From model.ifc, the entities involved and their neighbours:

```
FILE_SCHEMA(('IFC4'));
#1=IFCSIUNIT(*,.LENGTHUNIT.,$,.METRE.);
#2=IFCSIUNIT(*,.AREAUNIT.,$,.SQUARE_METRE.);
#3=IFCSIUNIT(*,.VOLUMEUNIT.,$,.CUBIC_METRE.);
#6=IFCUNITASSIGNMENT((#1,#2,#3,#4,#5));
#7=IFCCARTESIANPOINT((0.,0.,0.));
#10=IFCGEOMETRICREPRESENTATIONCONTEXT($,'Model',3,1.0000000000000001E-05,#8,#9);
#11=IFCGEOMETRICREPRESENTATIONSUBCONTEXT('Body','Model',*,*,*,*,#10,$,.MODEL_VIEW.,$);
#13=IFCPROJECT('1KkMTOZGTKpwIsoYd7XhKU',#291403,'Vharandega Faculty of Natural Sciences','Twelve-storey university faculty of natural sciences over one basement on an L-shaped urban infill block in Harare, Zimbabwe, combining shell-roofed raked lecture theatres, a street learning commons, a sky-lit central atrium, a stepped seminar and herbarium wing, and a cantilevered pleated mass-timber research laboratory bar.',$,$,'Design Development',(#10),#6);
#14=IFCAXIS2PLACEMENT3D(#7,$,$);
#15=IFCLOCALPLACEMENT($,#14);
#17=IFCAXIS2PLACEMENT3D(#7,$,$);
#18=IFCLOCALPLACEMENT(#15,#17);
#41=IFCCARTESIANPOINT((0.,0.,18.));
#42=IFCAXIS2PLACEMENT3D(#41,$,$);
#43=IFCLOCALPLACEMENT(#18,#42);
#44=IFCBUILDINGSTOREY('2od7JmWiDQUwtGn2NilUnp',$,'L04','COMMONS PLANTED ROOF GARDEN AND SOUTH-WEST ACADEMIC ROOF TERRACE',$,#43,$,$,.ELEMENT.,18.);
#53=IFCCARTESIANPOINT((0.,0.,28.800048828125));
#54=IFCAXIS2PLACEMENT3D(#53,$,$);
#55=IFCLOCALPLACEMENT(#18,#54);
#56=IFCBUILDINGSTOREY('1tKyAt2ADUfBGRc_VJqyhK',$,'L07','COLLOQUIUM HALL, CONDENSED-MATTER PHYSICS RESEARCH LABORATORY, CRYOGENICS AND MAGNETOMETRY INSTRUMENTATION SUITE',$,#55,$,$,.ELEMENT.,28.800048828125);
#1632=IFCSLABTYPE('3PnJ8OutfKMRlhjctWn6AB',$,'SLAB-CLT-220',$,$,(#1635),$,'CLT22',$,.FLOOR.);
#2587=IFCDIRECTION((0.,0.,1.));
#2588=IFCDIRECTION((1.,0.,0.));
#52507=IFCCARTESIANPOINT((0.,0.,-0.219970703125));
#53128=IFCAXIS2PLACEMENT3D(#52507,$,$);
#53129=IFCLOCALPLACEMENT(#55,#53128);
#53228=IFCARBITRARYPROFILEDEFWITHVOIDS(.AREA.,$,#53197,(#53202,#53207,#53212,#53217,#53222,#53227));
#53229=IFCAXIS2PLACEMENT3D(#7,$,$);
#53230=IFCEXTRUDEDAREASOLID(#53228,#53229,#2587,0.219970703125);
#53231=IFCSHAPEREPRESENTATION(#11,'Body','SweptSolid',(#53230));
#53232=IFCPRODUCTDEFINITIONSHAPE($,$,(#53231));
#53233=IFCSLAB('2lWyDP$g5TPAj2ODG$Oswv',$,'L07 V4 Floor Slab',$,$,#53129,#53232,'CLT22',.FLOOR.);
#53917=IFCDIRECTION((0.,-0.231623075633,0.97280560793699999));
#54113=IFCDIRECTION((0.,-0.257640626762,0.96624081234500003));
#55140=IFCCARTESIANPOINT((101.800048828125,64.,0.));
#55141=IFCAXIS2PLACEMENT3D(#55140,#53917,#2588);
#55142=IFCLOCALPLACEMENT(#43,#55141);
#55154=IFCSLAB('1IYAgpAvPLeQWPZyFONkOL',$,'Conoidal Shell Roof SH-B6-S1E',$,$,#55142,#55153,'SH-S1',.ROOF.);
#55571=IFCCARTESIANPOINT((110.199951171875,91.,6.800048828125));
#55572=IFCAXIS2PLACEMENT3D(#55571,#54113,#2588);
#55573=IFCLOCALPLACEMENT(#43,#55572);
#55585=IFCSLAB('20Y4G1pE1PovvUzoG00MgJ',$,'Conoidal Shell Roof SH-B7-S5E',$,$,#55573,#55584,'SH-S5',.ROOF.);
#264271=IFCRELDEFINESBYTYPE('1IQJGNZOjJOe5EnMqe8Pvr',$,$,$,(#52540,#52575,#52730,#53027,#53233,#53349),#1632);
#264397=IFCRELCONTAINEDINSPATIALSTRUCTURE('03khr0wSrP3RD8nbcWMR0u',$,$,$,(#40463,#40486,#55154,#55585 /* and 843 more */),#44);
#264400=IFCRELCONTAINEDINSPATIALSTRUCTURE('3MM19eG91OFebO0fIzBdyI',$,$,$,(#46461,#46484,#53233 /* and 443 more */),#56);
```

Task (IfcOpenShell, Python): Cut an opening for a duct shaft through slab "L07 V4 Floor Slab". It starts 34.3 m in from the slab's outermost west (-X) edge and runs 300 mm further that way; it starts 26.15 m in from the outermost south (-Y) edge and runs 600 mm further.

```python
import numpy as np
import ifcopenshell
import ifcopenshell.api.feature
import ifcopenshell.api.geometry
import ifcopenshell.api.root
import ifcopenshell.geom
import ifcopenshell.util.placement
import ifcopenshell.util.representation
import ifcopenshell.util.shape
import ifcopenshell.util.unit

model = ifcopenshell.open("model.ifc")
unit_scale = ifcopenshell.util.unit.calculate_unit_scale(model)
settings = ifcopenshell.geom.settings()


def volume(element):
    """Net volume in cubic metres, openings subtracted."""
    shape = ifcopenshell.geom.create_shape(settings, element)
    return ifcopenshell.util.shape.get_volume(shape.geometry)


slab = model.by_guid("2lWyDP$g5TPAj2ODG$Oswv")
before = volume(slab)

# Extent in the slab's own axes, in metres. The edges named are its -X and -Y sides.
slab_shape = ifcopenshell.geom.create_shape(settings, slab)
vertices = ifcopenshell.util.shape.get_vertices(slab_shape.geometry)
x_min, y_min, bottom = vertices.min(axis=0)
top = vertices[:, 2].max()

opening = ifcopenshell.api.root.create_entity(model, ifc_class="IfcOpeningElement", name="Duct shaft opening", predefined_type="OPENING")
context = ifcopenshell.util.representation.get_context(model, "Model", "Body", "MODEL_VIEW")
width, depth = 0.3, 0.6
outline = [(0.0, 0.0), (width, 0.0), (width, depth), (0.0, depth), (0.0, 0.0)]
# Overshoot both faces by 50 mm so the cut is clean.
shape = ifcopenshell.api.geometry.add_slab_representation(
    model, context=context, depth=top - bottom + 0.1, polyline=outline
)
ifcopenshell.api.geometry.assign_representation(model, product=opening, representation=shape)

matrix = ifcopenshell.util.placement.get_local_placement(slab.ObjectPlacement)
matrix[:, 3] = matrix @ np.append(np.array([x_min + 34.3, y_min + 26.15, bottom - 0.05]) / unit_scale, 1.0)
ifcopenshell.api.geometry.edit_object_placement(model, product=opening, matrix=matrix, is_si=False)
ifcopenshell.api.feature.add_feature(model, feature=opening, element=slab)

after = volume(slab)

print(f"slab volume {before:.3f} -> {after:.3f} m3")

model.write("model_edited.ifc")
```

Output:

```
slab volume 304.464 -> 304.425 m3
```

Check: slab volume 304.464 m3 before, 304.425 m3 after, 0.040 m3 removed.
